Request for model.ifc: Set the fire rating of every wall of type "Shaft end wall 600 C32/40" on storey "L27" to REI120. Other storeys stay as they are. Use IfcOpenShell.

First a look at what the model holds.

```python
import ifcopenshell
import ifcopenshell.util.element

model = ifcopenshell.open("model.ifc")
print(model.schema)
storey = next(s for s in model.by_type("IfcBuildingStorey") if s.Name == "L27")
walls = [e for e in ifcopenshell.util.element.get_decomposition(storey) if e.is_a("IfcWall")]
seen = {}
for e in walls:
    element_type = ifcopenshell.util.element.get_type(e)
    key = (element_type.Name if element_type != e and element_type else None, ifcopenshell.util.element.get_pset(e, "Pset_WallCommon", "FireRating"))
    seen[key] = seen.get(key, 0) + 1
for (name, value), count in sorted(seen.items(), key=str):
    print(count, "x", name, "|", value)
```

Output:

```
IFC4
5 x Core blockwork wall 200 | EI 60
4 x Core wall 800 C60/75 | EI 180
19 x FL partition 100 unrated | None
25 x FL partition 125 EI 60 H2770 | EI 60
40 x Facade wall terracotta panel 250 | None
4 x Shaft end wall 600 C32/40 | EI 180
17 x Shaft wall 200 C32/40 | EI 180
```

```python
import ifcopenshell
import ifcopenshell.api.pset
import ifcopenshell.util.element

model = ifcopenshell.open("model.ifc")

storey = next(s for s in model.by_type("IfcBuildingStorey") if s.Name == "L27")
walls = [e for e in ifcopenshell.util.element.get_decomposition(storey) if e.is_a("IfcWall")]

count = 0
for e in walls:
    element_type = ifcopenshell.util.element.get_type(e)
    if element_type in (None, e) or element_type.Name != "Shaft end wall 600 C32/40":
        continue
    found = ifcopenshell.util.element.get_pset(e, "Pset_WallCommon", should_inherit=False)
    if found:
        pset = model.by_id(found["id"])
        if len(ifcopenshell.util.element.get_elements_by_pset(pset)) > 1:
            pset = ifcopenshell.api.pset.unshare_pset(model, products=[e], pset=pset)[0]
    else:
        pset = ifcopenshell.api.pset.add_pset(model, product=e, name="Pset_WallCommon")
    ifcopenshell.api.pset.edit_pset(model, pset=pset, properties={"FireRating": "REI120"})
    count += 1

print(count, "walls updated")

model.write("model_updated.ifc")
```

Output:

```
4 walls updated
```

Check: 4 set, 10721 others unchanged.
